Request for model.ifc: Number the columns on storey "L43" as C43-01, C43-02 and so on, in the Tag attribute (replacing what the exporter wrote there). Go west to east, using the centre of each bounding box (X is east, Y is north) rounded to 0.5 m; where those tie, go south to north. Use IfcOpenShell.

First a look at what the model holds.

```python
import ifcopenshell
import ifcopenshell.util.element
import ifcopenshell.util.placement

model = ifcopenshell.open("model.ifc")
print(model.schema)
storey = next(s for s in model.by_type("IfcBuildingStorey") if s.Name == "L43")
columns = [e for e in ifcopenshell.util.element.get_decomposition(storey) if e.is_a("IfcColumn")]
for e in sorted(columns, key=lambda e: e.id()):
    origin = ifcopenshell.util.placement.get_local_placement(e.ObjectPlacement)[:3, 3]
    print(e.id(), e.Tag, e.Name, origin.round(2) + 0.0, sep=" | ")
```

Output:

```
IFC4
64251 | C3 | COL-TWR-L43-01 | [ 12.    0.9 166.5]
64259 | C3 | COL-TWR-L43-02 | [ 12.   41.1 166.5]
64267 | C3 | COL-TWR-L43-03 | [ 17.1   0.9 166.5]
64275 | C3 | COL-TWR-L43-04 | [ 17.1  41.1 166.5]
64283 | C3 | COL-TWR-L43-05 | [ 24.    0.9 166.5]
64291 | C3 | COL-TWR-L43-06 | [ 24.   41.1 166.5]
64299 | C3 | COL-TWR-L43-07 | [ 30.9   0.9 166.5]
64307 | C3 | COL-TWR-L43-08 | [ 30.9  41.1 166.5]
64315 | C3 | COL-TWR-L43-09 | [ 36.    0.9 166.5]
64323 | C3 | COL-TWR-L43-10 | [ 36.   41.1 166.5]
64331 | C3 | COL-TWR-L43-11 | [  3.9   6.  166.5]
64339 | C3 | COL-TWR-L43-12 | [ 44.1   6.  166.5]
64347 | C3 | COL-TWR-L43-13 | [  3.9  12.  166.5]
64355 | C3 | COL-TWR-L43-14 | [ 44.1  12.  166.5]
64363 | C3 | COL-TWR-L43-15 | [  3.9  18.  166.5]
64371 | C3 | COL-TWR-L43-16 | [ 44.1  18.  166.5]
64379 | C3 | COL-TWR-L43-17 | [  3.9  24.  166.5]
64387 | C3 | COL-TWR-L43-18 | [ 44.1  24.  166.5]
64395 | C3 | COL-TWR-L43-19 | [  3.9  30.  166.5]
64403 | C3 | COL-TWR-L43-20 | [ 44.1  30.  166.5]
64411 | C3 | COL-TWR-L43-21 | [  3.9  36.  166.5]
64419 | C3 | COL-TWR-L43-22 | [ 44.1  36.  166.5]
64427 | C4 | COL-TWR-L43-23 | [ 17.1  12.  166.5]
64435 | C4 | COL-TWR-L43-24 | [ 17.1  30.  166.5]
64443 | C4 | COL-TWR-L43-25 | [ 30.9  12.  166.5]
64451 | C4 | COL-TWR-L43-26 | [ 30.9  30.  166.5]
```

```python
import ifcopenshell
import ifcopenshell.geom
import ifcopenshell.util.element
import ifcopenshell.util.shape

model = ifcopenshell.open("model.ifc")
settings = ifcopenshell.geom.settings()
settings.set("use-world-coords", True)


def centre(element):
    shape = ifcopenshell.geom.create_shape(settings, element)
    return ifcopenshell.util.shape.get_bbox_centroid(shape.geometry)


storey = next(s for s in model.by_type("IfcBuildingStorey") if s.Name == "L43")
columns = [e for e in ifcopenshell.util.element.get_decomposition(storey) if e.is_a("IfcColumn")]

# Insertion points can sit at a corner or the storey origin, so sort by the geometry (in metres).
centres = {e: centre(e) for e in columns}
columns.sort(key=lambda e: (round(centres[e][0] / 0.5), centres[e][1]))

for i, e in enumerate(columns, start=1):
    number = f"C43-{i:02d}"
    e.Tag = number
    print(e.id(), number)

model.write("model_edited.ifc")
```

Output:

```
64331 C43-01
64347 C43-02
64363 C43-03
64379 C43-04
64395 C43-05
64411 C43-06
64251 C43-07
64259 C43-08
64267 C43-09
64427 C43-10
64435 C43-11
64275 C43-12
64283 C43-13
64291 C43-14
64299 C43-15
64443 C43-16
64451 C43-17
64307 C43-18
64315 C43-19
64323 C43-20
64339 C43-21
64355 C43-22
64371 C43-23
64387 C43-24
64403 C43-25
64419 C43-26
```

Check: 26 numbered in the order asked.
